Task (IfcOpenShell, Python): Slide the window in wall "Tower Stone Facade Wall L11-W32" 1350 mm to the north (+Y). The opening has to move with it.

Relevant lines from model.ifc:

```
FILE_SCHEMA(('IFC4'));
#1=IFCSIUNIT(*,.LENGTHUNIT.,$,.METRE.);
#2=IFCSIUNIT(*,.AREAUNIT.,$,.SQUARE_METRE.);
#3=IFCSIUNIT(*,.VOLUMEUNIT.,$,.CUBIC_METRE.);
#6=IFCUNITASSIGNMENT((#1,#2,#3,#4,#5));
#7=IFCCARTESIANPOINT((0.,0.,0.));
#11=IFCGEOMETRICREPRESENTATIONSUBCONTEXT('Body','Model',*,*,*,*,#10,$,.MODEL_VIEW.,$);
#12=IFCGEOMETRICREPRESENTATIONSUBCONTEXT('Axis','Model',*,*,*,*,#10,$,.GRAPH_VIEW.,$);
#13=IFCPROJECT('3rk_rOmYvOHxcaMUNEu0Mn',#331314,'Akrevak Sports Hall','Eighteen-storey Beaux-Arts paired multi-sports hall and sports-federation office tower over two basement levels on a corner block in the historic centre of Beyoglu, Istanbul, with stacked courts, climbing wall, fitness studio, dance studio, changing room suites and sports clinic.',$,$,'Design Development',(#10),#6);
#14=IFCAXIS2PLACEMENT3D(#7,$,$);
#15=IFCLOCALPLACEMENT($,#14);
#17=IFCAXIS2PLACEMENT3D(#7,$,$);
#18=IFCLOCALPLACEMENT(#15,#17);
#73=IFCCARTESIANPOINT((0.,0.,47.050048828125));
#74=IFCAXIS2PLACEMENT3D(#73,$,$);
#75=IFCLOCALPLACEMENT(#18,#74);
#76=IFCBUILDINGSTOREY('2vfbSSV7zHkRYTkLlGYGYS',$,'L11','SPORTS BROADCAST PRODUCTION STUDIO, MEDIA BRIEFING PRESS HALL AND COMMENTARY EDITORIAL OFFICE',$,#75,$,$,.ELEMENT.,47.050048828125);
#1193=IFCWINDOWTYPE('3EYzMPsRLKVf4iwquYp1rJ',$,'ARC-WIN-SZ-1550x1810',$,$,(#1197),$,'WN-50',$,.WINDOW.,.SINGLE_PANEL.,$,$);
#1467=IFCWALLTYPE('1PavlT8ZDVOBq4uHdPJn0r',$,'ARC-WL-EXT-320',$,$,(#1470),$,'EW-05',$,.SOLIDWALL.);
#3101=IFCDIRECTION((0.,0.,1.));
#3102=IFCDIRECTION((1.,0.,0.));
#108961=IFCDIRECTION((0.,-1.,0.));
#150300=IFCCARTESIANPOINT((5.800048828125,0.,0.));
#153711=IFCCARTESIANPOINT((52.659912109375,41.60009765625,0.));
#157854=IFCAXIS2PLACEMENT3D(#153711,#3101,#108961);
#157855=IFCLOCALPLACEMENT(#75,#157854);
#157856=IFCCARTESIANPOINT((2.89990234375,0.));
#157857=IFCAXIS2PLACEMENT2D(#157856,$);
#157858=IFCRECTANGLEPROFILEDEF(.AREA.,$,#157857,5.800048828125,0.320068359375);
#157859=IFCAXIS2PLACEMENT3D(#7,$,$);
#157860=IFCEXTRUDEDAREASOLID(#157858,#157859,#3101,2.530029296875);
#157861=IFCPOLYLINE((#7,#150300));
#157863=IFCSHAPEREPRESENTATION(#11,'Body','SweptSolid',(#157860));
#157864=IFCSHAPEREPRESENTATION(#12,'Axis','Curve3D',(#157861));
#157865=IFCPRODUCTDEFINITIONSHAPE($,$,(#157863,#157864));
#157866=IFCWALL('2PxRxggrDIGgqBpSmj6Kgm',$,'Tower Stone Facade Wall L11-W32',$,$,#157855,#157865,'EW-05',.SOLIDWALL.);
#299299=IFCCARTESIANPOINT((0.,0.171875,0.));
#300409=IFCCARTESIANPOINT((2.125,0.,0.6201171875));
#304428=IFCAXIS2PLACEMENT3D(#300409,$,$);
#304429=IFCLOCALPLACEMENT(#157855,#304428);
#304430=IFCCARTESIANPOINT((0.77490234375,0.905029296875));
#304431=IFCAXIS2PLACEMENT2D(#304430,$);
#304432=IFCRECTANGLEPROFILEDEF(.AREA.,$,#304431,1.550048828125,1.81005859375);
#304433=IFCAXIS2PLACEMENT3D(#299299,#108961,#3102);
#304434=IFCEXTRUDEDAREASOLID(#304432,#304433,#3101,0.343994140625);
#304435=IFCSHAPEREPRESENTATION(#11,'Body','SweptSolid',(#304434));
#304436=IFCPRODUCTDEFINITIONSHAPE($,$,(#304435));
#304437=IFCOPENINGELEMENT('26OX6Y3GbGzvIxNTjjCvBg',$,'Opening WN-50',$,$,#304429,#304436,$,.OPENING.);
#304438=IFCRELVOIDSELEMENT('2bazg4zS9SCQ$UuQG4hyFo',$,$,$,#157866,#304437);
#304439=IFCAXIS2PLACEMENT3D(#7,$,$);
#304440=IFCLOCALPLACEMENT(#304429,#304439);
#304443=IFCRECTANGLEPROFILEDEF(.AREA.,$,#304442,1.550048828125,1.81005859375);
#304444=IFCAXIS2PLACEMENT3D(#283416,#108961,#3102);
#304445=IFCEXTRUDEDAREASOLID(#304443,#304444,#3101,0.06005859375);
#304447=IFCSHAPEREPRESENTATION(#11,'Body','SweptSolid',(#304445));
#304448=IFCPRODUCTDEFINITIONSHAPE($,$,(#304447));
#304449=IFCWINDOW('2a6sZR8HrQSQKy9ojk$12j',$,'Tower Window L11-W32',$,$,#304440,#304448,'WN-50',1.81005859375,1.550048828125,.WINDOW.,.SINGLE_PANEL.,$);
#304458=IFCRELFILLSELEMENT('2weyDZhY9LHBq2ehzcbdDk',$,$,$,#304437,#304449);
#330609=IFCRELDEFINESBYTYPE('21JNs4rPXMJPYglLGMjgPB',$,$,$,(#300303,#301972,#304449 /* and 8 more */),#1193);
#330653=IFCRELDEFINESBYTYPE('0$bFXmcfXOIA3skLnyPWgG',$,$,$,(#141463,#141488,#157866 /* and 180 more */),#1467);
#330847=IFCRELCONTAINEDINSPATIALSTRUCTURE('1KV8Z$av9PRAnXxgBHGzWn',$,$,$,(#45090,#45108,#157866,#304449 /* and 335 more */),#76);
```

```python
import ifcopenshell
import ifcopenshell.api.geometry
import ifcopenshell.util.placement

model = ifcopenshell.open("model.ifc")

window = model.by_id(304449)
opening = window.FillsVoids[0].RelatingOpeningElement
wall = opening.VoidsElements[0].RelatingBuildingElement

wall_matrix = ifcopenshell.util.placement.get_local_placement(wall.ObjectPlacement)
shift = wall_matrix[:3, 0] * -1.35
before = ifcopenshell.util.placement.get_local_placement(window.ObjectPlacement)[:3, 3].copy()

# The window is placed relative to its opening, so it follows when the opening moves.
matrix = ifcopenshell.util.placement.get_local_placement(opening.ObjectPlacement)
matrix[:3, 3] += shift
ifcopenshell.api.geometry.edit_object_placement(
    model, product=opening, matrix=matrix, is_si=False, should_transform_children=True
)

after = ifcopenshell.util.placement.get_local_placement(window.ObjectPlacement)[:3, 3]
print("window moved by", (after - before).round(3) + 0.0)

model.write("model-out.ifc")
```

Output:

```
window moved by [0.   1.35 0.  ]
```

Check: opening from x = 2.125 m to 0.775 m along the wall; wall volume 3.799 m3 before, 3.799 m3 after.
